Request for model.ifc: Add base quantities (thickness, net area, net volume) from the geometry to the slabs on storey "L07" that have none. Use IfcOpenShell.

First a look at what the model holds.

```python
import ifcopenshell
import ifcopenshell.util.element
import ifcopenshell.util.unit

model = ifcopenshell.open("model.ifc")
print(model.schema)
for unit_type in ("LENGTHUNIT", "AREAUNIT", "VOLUMEUNIT"):
    print(unit_type, ifcopenshell.util.unit.calculate_unit_scale(model, unit_type))
storey = next(s for s in model.by_type("IfcBuildingStorey") if s.Name == "L07")
slabs = [e for e in ifcopenshell.util.element.get_decomposition(storey) if e.is_a("IfcSlab")]
for e in sorted(slabs, key=lambda e: e.id()):
    print(e.id(), e.is_a(), e.Name, list(ifcopenshell.util.element.get_psets(e, qtos_only=True)), sep=" | ")
```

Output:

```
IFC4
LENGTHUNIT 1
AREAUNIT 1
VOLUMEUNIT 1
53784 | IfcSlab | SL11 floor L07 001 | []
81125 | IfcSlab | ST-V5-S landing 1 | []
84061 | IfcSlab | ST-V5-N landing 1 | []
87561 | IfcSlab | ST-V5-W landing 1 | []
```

```python
import ifcopenshell
import ifcopenshell.api.pset
import ifcopenshell.geom
import ifcopenshell.util.element
import ifcopenshell.util.shape
import ifcopenshell.util.unit

model = ifcopenshell.open("model.ifc")
unit_scale = ifcopenshell.util.unit.calculate_unit_scale(model)
area_scale = ifcopenshell.util.unit.calculate_unit_scale(model, "AREAUNIT")
volume_scale = ifcopenshell.util.unit.calculate_unit_scale(model, "VOLUMEUNIT")
settings = ifcopenshell.geom.settings()

storey = next(s for s in model.by_type("IfcBuildingStorey") if s.Name == "L07")
slabs = [e for e in ifcopenshell.util.element.get_decomposition(storey) if e.is_a("IfcSlab")]

for e in sorted(slabs, key=lambda e: e.id()):
    if ifcopenshell.util.element.get_psets(e, qtos_only=True, should_inherit=False):
        continue
    # Geometry comes back in metres, in the element's own axes.
    shape = ifcopenshell.geom.create_shape(settings, e)
    values = {
        "Width": ifcopenshell.util.shape.get_z(shape.geometry) / unit_scale,
        "NetArea": ifcopenshell.util.shape.get_footprint_area(shape.geometry) / area_scale,
        "NetVolume": ifcopenshell.util.shape.get_volume(shape.geometry) / volume_scale,
    }
    qto = ifcopenshell.api.pset.add_qto(model, product=e, name="Qto_SlabBaseQuantities")
    ifcopenshell.api.pset.edit_qto(model, qto=qto, properties=values)
    print(e.id(), {k: round(v, 3) for k, v in values.items()})

model.write("model_updated.ifc")
```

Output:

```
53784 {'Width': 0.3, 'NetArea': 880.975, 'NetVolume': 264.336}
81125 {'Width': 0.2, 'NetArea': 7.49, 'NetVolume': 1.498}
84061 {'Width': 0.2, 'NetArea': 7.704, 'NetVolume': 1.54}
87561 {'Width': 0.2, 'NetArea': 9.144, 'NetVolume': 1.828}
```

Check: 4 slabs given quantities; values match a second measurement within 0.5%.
